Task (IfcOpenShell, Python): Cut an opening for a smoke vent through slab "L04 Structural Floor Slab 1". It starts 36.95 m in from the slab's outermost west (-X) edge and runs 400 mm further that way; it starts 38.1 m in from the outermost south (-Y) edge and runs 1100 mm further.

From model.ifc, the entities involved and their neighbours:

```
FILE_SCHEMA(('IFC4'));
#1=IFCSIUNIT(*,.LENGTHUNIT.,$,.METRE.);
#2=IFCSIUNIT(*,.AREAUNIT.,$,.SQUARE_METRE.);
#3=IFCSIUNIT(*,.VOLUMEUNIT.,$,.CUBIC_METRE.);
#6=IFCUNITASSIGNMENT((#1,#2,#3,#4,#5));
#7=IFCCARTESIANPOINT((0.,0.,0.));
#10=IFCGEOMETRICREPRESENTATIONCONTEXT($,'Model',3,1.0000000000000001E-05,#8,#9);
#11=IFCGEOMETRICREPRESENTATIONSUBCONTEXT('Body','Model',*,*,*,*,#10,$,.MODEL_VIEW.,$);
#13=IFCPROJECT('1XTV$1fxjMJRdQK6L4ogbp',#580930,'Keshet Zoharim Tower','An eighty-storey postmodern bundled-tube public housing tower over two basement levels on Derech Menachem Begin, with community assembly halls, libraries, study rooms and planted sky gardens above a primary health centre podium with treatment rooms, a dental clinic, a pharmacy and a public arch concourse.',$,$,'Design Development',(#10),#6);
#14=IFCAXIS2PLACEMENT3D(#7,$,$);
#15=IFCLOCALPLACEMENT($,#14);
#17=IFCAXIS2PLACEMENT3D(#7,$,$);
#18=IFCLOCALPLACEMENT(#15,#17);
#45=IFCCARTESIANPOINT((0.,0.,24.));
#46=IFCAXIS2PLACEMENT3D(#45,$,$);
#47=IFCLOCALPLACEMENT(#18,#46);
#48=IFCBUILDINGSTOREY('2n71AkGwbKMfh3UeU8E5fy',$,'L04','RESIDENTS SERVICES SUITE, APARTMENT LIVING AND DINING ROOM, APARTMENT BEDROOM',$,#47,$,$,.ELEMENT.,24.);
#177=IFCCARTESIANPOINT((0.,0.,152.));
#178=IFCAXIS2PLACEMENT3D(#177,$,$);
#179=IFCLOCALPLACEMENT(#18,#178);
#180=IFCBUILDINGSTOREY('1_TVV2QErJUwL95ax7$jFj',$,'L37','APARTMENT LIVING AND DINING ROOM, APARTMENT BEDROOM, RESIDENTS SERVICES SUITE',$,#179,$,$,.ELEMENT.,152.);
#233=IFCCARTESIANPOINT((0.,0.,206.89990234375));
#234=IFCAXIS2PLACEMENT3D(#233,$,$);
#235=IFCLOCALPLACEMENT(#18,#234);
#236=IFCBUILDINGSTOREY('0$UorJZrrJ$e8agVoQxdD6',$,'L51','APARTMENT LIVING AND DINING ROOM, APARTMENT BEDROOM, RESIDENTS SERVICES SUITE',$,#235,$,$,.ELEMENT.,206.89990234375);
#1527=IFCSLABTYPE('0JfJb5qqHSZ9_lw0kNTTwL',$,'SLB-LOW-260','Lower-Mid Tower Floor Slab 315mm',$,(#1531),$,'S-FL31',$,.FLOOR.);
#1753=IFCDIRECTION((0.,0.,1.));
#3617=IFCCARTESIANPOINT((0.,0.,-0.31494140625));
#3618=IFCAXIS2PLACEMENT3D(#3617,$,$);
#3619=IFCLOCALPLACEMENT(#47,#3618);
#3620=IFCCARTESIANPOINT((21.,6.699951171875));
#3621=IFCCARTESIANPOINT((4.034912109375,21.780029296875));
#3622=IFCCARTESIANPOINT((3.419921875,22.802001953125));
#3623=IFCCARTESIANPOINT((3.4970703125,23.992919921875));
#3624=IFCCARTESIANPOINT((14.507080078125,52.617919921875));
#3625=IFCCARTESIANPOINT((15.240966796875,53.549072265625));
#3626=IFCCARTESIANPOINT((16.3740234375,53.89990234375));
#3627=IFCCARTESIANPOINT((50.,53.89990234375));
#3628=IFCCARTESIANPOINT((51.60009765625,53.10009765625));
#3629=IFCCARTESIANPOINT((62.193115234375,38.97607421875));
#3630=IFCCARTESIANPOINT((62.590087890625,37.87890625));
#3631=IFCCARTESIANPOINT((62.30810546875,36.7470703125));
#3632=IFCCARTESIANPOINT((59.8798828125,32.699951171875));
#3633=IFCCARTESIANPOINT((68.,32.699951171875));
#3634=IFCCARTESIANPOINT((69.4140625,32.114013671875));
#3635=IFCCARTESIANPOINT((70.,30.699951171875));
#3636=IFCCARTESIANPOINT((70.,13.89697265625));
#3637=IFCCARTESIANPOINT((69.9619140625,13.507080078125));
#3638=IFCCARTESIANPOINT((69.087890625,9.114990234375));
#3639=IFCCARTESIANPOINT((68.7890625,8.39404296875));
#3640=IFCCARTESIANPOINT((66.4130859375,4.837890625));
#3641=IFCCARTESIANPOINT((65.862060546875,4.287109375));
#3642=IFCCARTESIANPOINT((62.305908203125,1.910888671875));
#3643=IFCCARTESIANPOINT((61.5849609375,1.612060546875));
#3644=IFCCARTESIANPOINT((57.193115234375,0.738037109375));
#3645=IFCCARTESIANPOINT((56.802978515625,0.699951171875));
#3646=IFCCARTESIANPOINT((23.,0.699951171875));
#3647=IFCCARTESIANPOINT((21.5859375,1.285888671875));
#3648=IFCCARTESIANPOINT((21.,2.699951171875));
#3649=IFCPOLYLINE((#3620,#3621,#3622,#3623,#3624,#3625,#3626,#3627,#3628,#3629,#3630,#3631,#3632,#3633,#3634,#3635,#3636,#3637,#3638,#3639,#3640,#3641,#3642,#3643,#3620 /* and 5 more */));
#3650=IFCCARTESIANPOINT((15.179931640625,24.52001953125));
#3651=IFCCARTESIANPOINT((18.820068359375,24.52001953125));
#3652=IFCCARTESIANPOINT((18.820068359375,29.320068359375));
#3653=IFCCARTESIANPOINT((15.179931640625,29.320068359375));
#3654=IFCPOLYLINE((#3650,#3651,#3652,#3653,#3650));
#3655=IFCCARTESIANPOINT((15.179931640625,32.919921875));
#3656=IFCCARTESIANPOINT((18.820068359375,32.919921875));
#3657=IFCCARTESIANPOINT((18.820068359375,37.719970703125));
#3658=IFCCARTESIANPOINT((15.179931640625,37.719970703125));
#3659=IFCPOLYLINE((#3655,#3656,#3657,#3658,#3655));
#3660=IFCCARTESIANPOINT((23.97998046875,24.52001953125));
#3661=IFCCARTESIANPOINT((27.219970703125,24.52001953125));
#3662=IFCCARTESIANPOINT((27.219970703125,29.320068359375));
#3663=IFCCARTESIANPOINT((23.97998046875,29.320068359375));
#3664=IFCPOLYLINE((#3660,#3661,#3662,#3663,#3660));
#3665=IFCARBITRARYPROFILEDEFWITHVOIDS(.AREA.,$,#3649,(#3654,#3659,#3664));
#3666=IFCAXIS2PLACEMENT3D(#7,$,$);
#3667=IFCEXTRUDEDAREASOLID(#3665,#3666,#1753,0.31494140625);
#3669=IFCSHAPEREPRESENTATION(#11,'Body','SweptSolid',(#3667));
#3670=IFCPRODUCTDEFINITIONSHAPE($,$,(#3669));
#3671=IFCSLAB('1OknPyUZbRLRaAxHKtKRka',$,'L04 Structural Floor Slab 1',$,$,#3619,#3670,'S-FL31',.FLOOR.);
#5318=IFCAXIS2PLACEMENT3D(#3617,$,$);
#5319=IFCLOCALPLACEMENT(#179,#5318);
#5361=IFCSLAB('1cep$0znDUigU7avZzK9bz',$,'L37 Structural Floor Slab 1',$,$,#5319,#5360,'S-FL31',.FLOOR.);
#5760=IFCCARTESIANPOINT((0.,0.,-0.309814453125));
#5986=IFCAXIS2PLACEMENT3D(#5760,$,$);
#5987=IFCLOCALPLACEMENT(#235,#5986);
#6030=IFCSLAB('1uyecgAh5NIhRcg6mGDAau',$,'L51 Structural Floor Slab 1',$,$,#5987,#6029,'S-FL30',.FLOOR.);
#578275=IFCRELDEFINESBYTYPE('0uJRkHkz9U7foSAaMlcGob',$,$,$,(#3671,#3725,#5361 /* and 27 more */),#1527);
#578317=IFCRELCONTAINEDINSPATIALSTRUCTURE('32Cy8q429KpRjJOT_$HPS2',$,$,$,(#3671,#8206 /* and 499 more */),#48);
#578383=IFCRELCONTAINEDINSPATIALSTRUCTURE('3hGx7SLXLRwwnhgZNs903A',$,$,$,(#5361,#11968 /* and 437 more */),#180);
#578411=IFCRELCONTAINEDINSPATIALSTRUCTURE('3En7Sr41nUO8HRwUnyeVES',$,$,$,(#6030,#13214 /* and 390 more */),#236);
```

```python
import numpy as np
import ifcopenshell
import ifcopenshell.api.feature
import ifcopenshell.api.geometry
import ifcopenshell.api.root
import ifcopenshell.geom
import ifcopenshell.util.placement
import ifcopenshell.util.representation
import ifcopenshell.util.shape
import ifcopenshell.util.unit

model = ifcopenshell.open("model.ifc")
unit_scale = ifcopenshell.util.unit.calculate_unit_scale(model)
settings = ifcopenshell.geom.settings()


def volume(element):
    """Net volume in cubic metres, openings subtracted."""
    shape = ifcopenshell.geom.create_shape(settings, element)
    return ifcopenshell.util.shape.get_volume(shape.geometry)


slab = model.by_id(3671)
before = volume(slab)

# Extent in the slab's own axes, in metres. The edges named are its -X and -Y sides.
slab_shape = ifcopenshell.geom.create_shape(settings, slab)
vertices = ifcopenshell.util.shape.get_vertices(slab_shape.geometry)
x_min, y_min, bottom = vertices.min(axis=0)
top = vertices[:, 2].max()

opening = ifcopenshell.api.root.create_entity(model, ifc_class="IfcOpeningElement", name="Smoke vent opening", predefined_type="OPENING")
context = ifcopenshell.util.representation.get_context(model, "Model", "Body", "MODEL_VIEW")
width, depth = 0.4, 1.1
outline = [(0.0, 0.0), (width, 0.0), (width, depth), (0.0, depth), (0.0, 0.0)]
# Overshoot both faces by 50 mm so the cut is clean.
shape = ifcopenshell.api.geometry.add_slab_representation(
    model, context=context, depth=top - bottom + 0.1, polyline=outline
)
ifcopenshell.api.geometry.assign_representation(model, product=opening, representation=shape)

matrix = ifcopenshell.util.placement.get_local_placement(slab.ObjectPlacement)
matrix[:, 3] = matrix @ np.append(np.array([x_min + 36.95, y_min + 38.1, bottom - 0.05]) / unit_scale, 1.0)
ifcopenshell.api.geometry.edit_object_placement(model, product=opening, matrix=matrix, is_si=False)
ifcopenshell.api.feature.add_feature(model, feature=opening, element=slab)

after = volume(slab)

print(f"slab volume {before:.3f} -> {after:.3f} m3")

model.write("model_rev.ifc")
```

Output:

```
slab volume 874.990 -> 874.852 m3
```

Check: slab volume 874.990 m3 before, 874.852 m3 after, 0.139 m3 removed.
